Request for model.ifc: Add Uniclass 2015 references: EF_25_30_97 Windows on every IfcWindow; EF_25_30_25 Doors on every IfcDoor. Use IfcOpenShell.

First a look at what the model holds.

```python
import ifcopenshell

model = ifcopenshell.open("model.ifc")
print(model.schema)
print("classifications:", [c.Name for c in model.by_type("IfcClassification")])
for ifc_class in ("IfcDoor", "IfcRoof", "IfcStair", "IfcWall", "IfcWindow"):
    print(ifc_class, len(model.by_type(ifc_class)))
```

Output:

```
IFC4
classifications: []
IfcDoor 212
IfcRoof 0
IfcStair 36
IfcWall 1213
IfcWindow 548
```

```python
import ifcopenshell
import ifcopenshell.api.classification

model = ifcopenshell.open("model.ifc")

system = ifcopenshell.api.classification.add_classification(model, classification="Uniclass 2015")

codes = {
    "IfcWindow": ("EF_25_30_97", "Windows"),
    "IfcDoor": ("EF_25_30_25", "Doors"),
}
for ifc_class, (code, name) in codes.items():
    products = model.by_type(ifc_class)
    ifcopenshell.api.classification.add_reference(
        model, products=products, classification=system, identification=code, name=name
    )
    print(code, len(products))

model.write("model-out.ifc")
```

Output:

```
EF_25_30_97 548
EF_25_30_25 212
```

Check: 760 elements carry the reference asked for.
